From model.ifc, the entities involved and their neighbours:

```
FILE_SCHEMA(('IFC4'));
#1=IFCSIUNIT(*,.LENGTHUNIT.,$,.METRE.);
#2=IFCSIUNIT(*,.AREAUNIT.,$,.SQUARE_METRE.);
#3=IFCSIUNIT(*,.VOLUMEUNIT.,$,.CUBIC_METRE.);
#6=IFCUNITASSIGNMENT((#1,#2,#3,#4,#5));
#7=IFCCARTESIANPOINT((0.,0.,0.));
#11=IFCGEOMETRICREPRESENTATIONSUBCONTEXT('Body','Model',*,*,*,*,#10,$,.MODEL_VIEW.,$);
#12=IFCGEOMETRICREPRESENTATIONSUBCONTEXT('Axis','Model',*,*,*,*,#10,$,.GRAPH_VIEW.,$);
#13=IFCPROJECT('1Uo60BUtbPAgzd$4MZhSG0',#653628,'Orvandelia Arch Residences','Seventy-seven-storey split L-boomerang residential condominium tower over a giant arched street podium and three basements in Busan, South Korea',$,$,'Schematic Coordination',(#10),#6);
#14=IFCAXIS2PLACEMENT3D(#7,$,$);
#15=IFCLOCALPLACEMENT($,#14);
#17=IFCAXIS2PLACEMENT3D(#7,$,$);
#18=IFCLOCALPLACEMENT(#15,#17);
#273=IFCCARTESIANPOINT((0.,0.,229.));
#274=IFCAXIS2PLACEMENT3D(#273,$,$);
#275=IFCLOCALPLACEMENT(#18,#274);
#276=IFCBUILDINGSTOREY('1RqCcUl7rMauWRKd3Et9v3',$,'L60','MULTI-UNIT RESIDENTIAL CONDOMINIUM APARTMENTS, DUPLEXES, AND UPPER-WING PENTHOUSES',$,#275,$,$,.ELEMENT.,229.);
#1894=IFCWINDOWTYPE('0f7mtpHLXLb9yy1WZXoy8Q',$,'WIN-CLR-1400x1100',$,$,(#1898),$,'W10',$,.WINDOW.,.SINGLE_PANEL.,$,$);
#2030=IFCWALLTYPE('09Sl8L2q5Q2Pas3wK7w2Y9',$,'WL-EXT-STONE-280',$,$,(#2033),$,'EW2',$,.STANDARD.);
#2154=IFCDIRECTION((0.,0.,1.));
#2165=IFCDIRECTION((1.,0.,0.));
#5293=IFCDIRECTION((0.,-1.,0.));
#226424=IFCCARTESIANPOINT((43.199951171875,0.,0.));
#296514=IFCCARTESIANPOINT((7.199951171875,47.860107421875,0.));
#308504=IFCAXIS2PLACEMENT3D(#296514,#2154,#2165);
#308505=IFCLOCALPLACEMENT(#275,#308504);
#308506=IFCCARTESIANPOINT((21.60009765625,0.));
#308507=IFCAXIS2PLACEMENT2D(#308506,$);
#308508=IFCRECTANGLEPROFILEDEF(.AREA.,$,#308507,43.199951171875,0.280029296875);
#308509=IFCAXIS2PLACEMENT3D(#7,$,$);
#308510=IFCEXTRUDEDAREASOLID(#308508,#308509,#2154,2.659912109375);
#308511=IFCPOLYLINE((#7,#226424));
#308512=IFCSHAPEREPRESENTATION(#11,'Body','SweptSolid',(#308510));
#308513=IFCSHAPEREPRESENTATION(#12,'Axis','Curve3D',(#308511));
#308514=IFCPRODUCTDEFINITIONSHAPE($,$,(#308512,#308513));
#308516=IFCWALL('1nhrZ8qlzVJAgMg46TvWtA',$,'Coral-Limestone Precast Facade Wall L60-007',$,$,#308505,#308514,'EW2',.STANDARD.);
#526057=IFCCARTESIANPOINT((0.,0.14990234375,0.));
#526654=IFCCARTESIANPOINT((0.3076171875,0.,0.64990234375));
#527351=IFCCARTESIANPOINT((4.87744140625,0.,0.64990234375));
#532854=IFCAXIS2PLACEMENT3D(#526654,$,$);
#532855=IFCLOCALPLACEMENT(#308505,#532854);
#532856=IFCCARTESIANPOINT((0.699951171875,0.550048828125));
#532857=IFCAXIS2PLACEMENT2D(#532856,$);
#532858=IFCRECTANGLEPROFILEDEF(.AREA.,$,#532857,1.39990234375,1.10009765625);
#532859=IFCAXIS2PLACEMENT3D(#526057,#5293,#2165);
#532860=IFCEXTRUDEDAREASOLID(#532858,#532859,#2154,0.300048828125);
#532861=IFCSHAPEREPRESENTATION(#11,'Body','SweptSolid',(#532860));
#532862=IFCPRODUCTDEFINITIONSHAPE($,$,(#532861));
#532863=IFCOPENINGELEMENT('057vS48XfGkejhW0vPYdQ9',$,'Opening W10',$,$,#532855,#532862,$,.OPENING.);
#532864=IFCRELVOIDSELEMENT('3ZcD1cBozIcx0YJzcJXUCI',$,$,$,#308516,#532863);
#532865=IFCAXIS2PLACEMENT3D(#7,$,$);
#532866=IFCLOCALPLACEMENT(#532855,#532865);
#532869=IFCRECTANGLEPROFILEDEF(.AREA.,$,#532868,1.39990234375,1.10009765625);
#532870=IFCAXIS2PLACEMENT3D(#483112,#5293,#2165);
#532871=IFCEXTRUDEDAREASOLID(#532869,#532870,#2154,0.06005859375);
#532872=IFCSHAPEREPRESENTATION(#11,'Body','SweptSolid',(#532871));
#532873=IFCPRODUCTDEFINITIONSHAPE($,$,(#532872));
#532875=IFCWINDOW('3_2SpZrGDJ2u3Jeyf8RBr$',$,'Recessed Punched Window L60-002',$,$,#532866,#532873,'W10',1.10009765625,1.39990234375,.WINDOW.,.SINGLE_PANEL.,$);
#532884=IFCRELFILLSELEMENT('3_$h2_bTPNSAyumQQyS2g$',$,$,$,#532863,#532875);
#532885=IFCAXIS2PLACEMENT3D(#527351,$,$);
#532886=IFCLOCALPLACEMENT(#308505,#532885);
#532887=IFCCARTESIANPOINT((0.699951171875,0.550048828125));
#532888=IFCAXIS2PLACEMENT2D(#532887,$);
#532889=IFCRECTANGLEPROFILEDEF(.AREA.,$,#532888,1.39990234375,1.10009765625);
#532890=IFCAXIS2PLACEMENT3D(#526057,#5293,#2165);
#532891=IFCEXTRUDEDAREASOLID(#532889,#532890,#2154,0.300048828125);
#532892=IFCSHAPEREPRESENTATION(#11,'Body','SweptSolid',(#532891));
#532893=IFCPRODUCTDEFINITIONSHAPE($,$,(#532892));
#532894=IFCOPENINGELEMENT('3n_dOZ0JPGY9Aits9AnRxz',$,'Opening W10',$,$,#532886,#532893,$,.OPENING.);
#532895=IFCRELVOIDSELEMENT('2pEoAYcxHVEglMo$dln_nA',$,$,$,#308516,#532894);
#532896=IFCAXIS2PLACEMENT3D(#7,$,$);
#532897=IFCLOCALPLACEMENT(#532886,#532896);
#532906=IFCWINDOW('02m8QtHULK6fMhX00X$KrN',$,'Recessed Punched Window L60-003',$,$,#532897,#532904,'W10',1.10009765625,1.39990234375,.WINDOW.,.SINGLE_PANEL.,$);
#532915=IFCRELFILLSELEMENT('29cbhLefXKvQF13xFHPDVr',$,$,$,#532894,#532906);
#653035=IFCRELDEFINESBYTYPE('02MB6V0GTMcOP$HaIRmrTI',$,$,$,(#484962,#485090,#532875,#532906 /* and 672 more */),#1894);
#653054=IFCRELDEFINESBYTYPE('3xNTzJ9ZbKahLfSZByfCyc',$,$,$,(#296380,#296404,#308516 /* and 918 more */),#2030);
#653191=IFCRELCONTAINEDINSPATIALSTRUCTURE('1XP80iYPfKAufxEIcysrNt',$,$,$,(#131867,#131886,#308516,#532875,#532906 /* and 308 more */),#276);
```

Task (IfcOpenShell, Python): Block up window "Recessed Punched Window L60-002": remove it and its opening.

```python
import ifcopenshell
import ifcopenshell.api.feature
import ifcopenshell.api.root
import ifcopenshell.geom
import ifcopenshell.util.shape

model = ifcopenshell.open("model.ifc")
settings = ifcopenshell.geom.settings()


def volume(element):
    """Net volume in cubic metres, openings subtracted."""
    shape = ifcopenshell.geom.create_shape(settings, element)
    return ifcopenshell.util.shape.get_volume(shape.geometry)


window = model.by_id(532875)
opening = window.FillsVoids[0].RelatingOpeningElement
wall = opening.VoidsElements[0].RelatingBuildingElement
before = volume(wall)

ifcopenshell.api.root.remove_product(model, product=window)
ifcopenshell.api.feature.remove_feature(model, feature=opening)

after = volume(wall)

print(f"wall volume {before:.3f} -> {after:.3f} m3")

model.write("model_updated.ifc")
```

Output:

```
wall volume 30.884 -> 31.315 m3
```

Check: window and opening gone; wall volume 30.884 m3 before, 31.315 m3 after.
